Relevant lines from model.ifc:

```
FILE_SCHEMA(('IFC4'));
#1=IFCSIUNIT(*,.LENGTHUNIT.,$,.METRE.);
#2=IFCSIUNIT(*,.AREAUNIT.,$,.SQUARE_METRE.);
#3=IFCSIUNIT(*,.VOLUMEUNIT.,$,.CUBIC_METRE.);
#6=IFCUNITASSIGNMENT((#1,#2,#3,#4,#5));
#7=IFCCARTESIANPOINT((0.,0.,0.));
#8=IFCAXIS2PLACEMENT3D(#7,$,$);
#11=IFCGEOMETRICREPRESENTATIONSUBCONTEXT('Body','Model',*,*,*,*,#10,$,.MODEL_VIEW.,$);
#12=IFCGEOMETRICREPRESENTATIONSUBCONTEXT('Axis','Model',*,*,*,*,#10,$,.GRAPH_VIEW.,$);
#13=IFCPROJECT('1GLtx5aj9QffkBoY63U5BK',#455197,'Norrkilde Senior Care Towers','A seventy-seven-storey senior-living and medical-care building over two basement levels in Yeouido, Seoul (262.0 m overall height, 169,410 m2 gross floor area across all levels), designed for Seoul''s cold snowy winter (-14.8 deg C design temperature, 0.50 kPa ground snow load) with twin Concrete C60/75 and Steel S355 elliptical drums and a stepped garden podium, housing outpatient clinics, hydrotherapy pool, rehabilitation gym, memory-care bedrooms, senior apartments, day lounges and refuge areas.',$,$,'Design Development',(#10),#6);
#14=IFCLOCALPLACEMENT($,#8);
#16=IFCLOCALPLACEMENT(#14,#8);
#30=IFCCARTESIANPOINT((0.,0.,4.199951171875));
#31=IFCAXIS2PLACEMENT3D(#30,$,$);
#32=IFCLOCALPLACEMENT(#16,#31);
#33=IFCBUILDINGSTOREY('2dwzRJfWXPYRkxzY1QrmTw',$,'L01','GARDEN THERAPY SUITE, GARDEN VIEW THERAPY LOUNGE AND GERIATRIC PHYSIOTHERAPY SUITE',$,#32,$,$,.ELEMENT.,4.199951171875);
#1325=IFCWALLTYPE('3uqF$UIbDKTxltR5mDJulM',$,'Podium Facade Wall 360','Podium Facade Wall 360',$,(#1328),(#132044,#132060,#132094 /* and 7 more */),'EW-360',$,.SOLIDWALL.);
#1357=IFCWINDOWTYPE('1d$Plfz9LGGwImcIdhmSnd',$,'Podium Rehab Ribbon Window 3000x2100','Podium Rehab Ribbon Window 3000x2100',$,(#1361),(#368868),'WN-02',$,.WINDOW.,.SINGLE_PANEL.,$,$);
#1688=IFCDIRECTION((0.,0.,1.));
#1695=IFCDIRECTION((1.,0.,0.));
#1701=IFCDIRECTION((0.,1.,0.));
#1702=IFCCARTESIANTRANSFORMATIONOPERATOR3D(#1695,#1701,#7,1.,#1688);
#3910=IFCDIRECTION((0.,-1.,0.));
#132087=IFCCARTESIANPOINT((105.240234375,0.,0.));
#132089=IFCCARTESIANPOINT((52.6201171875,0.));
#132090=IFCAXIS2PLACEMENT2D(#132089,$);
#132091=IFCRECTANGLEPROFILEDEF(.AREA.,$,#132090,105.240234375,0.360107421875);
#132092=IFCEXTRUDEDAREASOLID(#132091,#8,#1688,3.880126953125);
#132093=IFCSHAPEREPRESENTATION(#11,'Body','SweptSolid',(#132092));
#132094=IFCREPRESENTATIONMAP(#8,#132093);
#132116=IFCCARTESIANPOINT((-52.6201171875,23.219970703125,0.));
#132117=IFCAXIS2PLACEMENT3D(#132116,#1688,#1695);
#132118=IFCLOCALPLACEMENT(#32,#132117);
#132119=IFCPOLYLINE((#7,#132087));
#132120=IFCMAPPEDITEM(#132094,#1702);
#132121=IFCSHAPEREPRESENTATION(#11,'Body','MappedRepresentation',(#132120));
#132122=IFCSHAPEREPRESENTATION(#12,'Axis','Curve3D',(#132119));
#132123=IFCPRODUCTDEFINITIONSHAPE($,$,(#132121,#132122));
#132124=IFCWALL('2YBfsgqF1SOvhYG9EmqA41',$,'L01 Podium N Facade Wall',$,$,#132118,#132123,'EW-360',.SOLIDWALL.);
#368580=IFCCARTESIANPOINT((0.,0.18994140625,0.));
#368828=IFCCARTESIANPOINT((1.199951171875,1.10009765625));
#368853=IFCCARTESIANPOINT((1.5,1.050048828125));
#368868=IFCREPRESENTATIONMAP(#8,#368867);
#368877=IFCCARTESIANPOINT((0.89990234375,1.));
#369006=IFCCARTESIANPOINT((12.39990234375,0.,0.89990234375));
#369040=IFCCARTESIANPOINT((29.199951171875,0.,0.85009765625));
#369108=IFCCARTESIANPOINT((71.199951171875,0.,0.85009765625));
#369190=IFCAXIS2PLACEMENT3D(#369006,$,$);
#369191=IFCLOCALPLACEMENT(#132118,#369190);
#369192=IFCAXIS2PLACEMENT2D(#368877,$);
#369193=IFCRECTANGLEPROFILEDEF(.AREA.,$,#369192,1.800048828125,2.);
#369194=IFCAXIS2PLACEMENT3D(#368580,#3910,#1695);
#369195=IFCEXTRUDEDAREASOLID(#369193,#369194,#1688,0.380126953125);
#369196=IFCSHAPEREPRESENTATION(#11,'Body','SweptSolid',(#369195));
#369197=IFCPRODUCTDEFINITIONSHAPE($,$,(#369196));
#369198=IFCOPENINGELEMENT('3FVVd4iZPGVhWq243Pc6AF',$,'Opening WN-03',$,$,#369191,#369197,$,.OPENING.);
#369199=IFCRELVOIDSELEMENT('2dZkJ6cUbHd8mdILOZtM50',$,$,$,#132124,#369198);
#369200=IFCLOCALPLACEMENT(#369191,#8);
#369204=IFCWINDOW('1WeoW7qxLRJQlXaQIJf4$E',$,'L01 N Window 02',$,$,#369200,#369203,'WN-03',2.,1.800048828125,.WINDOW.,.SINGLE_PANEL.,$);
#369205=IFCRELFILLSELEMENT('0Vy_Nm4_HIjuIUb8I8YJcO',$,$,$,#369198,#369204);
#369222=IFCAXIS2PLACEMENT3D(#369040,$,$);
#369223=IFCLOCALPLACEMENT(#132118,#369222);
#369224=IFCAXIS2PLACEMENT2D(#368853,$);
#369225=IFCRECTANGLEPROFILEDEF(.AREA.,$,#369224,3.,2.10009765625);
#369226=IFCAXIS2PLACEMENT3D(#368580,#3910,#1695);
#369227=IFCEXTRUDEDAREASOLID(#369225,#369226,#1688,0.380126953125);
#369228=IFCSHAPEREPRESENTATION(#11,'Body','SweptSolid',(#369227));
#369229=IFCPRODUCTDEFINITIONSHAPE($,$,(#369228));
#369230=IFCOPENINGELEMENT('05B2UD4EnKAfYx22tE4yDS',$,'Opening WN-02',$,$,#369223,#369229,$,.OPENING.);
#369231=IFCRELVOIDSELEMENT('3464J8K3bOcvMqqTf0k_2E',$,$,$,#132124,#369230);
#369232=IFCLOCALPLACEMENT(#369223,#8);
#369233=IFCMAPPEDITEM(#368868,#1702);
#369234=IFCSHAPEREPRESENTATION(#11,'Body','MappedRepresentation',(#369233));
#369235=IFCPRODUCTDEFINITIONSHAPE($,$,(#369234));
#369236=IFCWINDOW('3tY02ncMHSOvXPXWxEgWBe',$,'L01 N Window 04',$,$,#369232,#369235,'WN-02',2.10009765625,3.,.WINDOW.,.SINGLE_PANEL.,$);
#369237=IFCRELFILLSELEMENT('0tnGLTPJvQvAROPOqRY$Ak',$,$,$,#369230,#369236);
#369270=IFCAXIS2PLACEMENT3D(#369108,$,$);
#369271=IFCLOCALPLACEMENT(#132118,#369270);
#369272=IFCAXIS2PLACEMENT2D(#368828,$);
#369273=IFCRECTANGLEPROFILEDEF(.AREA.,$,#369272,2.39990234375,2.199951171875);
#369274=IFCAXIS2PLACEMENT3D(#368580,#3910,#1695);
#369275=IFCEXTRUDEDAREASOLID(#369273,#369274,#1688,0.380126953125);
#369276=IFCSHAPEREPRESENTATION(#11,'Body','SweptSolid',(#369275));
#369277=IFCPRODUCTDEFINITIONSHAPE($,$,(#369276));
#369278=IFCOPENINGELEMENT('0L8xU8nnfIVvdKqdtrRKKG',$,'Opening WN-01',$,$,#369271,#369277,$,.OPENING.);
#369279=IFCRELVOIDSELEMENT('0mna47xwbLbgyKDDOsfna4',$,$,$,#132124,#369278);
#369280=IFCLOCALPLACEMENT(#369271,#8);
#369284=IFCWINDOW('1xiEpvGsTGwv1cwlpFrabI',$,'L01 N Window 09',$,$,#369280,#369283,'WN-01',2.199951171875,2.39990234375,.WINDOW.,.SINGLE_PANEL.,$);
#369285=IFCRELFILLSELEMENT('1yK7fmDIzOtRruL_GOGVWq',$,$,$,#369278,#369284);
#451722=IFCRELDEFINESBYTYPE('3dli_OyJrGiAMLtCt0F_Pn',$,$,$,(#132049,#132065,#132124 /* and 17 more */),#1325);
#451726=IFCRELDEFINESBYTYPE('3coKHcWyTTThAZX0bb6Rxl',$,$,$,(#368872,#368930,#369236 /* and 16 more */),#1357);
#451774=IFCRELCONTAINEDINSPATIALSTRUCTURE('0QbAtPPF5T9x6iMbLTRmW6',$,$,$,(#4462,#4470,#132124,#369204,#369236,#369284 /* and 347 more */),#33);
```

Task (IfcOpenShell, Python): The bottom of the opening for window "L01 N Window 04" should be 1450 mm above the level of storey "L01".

```python
import numpy as np
import ifcopenshell
import ifcopenshell.api.geometry
import ifcopenshell.geom
import ifcopenshell.util.element
import ifcopenshell.util.placement
import ifcopenshell.util.shape
import ifcopenshell.util.unit

model = ifcopenshell.open("model.ifc")
unit_scale = ifcopenshell.util.unit.calculate_unit_scale(model)

window = model.by_guid("3tY02ncMHSOvXPXWxEgWBe")
opening = window.FillsVoids[0].RelatingOpeningElement
storey = ifcopenshell.util.element.get_container(window, ifc_class="IfcBuildingStorey")
level = ifcopenshell.util.placement.get_local_placement(storey.ObjectPlacement)[2, 3]

# The opening's origin need not be at the sill, so measure its lowest point.
shape = ifcopenshell.geom.create_shape(ifcopenshell.geom.settings(), opening)
bottom = ifcopenshell.util.shape.get_shape_bottom_elevation(shape, shape.geometry) / unit_scale
dz = level + 1.45 / unit_scale - bottom

shift = np.array([0.0, 0.0, dz])
# The window is placed relative to its opening, so it follows when the opening moves.
matrix = ifcopenshell.util.placement.get_local_placement(opening.ObjectPlacement)
matrix[:3, 3] += shift
ifcopenshell.api.geometry.edit_object_placement(
    model, product=opening, matrix=matrix, is_si=False, should_transform_children=True
)

print(f"moved by {dz * unit_scale:+.3f} m")

model.write("model_edited.ifc")
```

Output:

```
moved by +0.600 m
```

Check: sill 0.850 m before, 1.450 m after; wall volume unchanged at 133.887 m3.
